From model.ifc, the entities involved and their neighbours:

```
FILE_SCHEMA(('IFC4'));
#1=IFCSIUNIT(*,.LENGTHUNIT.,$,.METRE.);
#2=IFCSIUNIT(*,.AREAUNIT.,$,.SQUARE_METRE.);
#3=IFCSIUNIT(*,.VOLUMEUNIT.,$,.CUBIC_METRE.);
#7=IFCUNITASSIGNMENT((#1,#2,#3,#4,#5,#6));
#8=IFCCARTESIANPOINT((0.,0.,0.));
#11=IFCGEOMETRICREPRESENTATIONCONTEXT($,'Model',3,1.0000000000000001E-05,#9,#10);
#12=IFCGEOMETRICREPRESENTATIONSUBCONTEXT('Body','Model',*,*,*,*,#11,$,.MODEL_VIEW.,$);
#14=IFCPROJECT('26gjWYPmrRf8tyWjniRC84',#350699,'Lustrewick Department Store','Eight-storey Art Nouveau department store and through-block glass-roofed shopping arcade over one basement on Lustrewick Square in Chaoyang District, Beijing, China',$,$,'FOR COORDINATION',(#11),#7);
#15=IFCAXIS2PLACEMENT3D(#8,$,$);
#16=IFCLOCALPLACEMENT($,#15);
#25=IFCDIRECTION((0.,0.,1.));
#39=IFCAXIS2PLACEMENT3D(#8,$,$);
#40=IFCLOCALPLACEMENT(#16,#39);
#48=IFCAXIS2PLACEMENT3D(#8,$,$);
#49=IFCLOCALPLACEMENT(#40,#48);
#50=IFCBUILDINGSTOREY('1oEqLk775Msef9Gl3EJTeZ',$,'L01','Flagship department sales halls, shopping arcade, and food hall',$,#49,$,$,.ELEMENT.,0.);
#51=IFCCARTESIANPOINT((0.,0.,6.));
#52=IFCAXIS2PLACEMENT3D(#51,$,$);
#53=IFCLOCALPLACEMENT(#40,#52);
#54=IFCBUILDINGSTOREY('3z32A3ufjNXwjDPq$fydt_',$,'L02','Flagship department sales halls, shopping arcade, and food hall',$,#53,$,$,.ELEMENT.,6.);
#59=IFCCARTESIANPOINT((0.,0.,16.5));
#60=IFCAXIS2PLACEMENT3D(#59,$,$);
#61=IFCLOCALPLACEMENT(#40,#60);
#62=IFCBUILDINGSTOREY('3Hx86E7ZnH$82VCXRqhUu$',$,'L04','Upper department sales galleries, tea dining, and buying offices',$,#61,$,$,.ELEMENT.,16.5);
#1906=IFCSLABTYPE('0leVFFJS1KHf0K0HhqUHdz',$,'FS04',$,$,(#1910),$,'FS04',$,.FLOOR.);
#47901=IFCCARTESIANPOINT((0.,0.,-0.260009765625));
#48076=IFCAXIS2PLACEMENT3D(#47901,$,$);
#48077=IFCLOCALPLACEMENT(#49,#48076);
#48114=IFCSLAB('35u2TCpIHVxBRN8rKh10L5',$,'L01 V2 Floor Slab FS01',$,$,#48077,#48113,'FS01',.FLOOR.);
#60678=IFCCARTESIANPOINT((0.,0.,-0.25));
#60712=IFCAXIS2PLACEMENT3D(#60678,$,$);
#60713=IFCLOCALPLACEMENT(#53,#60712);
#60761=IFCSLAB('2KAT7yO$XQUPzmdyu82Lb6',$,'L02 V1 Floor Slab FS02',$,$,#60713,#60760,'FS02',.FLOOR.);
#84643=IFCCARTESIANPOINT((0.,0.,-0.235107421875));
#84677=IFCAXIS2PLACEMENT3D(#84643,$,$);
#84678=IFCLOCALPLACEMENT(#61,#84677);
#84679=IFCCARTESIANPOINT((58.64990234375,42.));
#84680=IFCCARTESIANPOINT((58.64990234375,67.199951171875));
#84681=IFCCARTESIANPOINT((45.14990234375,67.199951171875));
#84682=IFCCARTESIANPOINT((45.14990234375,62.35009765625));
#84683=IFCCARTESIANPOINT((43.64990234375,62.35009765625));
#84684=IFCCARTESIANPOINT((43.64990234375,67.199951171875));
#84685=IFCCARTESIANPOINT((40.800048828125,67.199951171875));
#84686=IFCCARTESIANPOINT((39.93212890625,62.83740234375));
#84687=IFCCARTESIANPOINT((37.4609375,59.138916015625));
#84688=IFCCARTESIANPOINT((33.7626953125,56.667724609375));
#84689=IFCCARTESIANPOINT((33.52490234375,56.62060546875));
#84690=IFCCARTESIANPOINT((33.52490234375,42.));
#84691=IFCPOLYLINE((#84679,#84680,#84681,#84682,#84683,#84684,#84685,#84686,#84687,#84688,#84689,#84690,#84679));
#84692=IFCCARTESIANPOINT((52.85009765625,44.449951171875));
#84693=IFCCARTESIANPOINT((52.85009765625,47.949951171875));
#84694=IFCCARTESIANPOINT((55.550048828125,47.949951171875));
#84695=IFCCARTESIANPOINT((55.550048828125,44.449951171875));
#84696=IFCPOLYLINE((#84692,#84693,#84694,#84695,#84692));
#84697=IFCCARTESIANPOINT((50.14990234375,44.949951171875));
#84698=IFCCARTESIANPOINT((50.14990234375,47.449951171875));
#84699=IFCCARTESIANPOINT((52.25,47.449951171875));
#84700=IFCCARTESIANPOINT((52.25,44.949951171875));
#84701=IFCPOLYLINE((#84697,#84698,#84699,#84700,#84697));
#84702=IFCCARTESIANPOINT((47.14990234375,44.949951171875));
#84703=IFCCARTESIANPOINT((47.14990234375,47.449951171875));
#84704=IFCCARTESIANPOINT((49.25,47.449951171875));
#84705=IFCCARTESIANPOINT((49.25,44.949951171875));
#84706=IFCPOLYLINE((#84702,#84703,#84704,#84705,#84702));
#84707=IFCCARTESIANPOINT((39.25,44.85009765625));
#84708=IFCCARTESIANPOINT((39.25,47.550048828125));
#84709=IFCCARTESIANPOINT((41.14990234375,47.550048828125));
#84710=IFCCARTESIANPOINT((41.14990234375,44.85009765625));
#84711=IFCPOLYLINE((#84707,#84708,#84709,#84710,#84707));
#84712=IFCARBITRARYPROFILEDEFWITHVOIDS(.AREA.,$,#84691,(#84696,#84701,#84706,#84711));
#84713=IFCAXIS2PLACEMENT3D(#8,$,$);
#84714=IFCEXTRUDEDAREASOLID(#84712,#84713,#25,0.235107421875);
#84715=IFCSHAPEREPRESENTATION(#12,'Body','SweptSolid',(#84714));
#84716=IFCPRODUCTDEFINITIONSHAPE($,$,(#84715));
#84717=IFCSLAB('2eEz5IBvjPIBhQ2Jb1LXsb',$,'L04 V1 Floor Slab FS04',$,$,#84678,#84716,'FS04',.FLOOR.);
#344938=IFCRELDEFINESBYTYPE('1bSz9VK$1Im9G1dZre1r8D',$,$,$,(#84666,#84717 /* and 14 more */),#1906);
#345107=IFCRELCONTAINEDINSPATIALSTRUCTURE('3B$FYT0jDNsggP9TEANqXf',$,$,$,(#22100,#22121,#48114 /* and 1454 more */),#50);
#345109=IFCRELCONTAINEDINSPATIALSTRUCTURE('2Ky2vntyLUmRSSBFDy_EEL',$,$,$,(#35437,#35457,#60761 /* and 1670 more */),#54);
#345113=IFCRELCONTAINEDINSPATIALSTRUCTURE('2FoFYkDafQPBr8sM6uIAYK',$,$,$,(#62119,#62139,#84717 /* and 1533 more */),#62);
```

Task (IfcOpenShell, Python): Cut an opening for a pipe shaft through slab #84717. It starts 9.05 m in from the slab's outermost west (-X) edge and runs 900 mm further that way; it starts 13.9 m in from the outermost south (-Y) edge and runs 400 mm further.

```python
import numpy as np
import ifcopenshell
import ifcopenshell.api.feature
import ifcopenshell.api.geometry
import ifcopenshell.api.root
import ifcopenshell.geom
import ifcopenshell.util.placement
import ifcopenshell.util.representation
import ifcopenshell.util.shape
import ifcopenshell.util.unit

model = ifcopenshell.open("model.ifc")
unit_scale = ifcopenshell.util.unit.calculate_unit_scale(model)
settings = ifcopenshell.geom.settings()


def volume(element):
    """Net volume in cubic metres, openings subtracted."""
    shape = ifcopenshell.geom.create_shape(settings, element)
    return ifcopenshell.util.shape.get_volume(shape.geometry)


slab = model.by_guid("2eEz5IBvjPIBhQ2Jb1LXsb")
before = volume(slab)

# Extent in the slab's own axes, in metres. The edges named are its -X and -Y sides.
slab_shape = ifcopenshell.geom.create_shape(settings, slab)
vertices = ifcopenshell.util.shape.get_vertices(slab_shape.geometry)
x_min, y_min, bottom = vertices.min(axis=0)
top = vertices[:, 2].max()

opening = ifcopenshell.api.root.create_entity(model, ifc_class="IfcOpeningElement", name="Pipe shaft opening", predefined_type="OPENING")
context = ifcopenshell.util.representation.get_context(model, "Model", "Body", "MODEL_VIEW")
width, depth = 0.9, 0.4
outline = [(0.0, 0.0), (width, 0.0), (width, depth), (0.0, depth), (0.0, 0.0)]
# Overshoot both faces by 50 mm so the cut is clean.
shape = ifcopenshell.api.geometry.add_slab_representation(
    model, context=context, depth=top - bottom + 0.1, polyline=outline
)
ifcopenshell.api.geometry.assign_representation(model, product=opening, representation=shape)

matrix = ifcopenshell.util.placement.get_local_placement(slab.ObjectPlacement)
matrix[:, 3] = matrix @ np.append(np.array([x_min + 9.05, y_min + 13.9, bottom - 0.05]) / unit_scale, 1.0)
ifcopenshell.api.geometry.edit_object_placement(model, product=opening, matrix=matrix, is_si=False)
ifcopenshell.api.feature.add_feature(model, feature=opening, element=slab)

after = volume(slab)

print(f"slab volume {before:.3f} -> {after:.3f} m3")

model.write("model_v2.ifc")
```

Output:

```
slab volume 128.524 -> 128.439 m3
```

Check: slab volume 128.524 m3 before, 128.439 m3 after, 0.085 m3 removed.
